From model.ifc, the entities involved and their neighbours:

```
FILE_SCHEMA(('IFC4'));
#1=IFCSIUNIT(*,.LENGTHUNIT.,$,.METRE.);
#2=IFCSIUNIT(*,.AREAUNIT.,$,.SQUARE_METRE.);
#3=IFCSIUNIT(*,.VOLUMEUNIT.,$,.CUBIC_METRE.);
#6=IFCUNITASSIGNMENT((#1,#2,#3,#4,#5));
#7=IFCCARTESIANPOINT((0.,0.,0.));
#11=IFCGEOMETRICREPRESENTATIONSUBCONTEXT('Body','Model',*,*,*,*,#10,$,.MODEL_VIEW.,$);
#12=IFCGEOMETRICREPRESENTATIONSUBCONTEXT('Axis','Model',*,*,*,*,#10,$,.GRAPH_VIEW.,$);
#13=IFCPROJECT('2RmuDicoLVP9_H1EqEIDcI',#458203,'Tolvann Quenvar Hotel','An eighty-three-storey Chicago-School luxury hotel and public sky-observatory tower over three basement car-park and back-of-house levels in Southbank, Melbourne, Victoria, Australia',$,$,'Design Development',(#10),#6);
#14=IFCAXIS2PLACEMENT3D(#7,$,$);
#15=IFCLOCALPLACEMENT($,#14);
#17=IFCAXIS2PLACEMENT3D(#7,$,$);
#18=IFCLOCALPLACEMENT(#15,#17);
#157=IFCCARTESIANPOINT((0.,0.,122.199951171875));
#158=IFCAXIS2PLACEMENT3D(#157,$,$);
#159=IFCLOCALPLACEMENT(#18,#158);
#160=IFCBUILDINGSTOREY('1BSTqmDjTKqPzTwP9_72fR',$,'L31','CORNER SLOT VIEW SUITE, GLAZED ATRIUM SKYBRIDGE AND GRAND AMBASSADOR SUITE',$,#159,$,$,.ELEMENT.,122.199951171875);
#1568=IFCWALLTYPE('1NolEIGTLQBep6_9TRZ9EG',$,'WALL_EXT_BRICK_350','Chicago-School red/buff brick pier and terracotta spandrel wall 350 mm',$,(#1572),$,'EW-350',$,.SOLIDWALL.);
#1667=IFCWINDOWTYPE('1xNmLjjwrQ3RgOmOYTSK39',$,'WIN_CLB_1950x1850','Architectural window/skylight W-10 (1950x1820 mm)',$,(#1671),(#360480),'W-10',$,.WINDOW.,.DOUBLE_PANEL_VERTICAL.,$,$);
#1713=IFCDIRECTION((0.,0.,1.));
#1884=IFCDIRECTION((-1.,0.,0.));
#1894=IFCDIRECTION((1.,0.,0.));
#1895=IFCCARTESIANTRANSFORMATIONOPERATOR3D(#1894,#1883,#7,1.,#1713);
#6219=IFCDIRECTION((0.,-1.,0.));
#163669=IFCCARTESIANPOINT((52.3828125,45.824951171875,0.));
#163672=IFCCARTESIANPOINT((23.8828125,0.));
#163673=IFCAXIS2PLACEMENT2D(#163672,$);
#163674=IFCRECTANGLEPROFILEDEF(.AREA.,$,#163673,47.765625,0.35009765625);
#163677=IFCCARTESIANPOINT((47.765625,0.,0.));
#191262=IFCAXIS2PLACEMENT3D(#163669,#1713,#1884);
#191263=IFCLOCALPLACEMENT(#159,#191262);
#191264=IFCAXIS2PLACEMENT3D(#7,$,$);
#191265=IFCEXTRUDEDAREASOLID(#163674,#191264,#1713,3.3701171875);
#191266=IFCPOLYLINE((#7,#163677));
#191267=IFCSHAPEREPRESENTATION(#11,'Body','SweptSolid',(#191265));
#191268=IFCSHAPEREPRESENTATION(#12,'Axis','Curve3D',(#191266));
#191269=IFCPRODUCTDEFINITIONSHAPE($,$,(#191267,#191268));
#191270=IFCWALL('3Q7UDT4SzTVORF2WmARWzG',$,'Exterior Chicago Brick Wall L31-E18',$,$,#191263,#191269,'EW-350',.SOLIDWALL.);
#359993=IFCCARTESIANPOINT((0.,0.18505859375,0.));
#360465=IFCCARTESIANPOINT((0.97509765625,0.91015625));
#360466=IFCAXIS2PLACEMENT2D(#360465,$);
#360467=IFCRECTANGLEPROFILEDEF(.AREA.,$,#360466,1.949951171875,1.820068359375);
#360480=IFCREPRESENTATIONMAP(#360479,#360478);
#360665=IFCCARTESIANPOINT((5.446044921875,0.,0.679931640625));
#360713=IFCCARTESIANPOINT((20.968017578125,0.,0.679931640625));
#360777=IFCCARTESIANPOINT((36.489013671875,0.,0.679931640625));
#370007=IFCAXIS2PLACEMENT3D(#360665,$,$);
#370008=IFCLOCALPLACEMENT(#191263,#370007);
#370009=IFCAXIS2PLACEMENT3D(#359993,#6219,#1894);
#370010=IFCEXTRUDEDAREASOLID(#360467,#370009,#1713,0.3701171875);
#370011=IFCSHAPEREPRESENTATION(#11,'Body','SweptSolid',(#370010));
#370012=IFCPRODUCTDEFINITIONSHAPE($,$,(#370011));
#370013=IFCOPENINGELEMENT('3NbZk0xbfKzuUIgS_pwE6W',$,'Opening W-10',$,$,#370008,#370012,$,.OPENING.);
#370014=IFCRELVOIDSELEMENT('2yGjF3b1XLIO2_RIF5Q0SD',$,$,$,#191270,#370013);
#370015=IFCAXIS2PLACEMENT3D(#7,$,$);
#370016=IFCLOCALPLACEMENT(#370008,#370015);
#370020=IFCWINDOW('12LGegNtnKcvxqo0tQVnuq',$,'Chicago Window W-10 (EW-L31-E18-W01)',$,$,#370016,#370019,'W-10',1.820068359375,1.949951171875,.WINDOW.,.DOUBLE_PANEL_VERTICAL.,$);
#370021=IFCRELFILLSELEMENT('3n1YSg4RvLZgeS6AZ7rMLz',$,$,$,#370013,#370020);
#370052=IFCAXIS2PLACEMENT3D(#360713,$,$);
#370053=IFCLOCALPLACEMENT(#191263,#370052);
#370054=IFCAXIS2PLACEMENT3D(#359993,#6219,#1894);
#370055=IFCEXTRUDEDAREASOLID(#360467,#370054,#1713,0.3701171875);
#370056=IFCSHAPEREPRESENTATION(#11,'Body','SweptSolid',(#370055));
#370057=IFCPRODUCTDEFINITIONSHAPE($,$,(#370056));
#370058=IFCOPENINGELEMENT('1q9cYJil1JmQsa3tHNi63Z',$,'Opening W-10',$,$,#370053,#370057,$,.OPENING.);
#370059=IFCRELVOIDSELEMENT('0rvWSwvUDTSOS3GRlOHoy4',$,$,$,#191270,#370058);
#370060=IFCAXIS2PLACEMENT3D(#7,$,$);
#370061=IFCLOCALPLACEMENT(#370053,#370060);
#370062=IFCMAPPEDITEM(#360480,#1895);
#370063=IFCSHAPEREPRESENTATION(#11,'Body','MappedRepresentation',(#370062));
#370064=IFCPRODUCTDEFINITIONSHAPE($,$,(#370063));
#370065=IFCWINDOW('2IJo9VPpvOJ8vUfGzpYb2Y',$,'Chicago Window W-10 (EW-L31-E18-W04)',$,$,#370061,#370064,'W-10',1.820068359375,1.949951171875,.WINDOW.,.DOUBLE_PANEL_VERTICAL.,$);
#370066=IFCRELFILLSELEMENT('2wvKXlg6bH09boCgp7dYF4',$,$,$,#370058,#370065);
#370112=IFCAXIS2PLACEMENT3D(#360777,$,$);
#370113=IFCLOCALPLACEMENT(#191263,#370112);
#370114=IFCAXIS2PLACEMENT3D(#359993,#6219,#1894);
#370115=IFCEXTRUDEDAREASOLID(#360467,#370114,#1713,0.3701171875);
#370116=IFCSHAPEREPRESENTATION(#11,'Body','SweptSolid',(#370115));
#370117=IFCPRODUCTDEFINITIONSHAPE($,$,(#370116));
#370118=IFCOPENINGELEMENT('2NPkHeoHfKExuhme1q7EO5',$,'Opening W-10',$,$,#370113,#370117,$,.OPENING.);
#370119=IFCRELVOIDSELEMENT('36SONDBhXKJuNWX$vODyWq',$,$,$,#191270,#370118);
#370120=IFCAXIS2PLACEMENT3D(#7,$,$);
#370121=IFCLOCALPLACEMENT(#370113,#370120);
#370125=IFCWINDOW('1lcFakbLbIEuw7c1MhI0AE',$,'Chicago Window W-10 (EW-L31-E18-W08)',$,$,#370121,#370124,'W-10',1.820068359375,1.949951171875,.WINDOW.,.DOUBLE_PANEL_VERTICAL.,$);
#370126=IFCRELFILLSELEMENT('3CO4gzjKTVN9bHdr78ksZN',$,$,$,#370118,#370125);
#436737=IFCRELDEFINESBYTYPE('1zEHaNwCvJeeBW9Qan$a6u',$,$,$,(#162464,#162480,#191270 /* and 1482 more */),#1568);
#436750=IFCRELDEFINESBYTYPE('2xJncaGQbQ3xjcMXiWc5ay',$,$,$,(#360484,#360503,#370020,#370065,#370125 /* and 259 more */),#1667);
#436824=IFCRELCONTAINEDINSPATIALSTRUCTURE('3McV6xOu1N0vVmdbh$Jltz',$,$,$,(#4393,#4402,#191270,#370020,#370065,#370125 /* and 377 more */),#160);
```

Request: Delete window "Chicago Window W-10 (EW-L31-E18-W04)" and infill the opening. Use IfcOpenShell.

```python
import ifcopenshell
import ifcopenshell.api.feature
import ifcopenshell.api.root
import ifcopenshell.geom
import ifcopenshell.util.shape

model = ifcopenshell.open("model.ifc")
settings = ifcopenshell.geom.settings()


def volume(element):
    """Net volume in cubic metres, openings subtracted."""
    shape = ifcopenshell.geom.create_shape(settings, element)
    return ifcopenshell.util.shape.get_volume(shape.geometry)


window = model.by_guid("2IJo9VPpvOJ8vUfGzpYb2Y")
opening = window.FillsVoids[0].RelatingOpeningElement
wall = opening.VoidsElements[0].RelatingBuildingElement
before = volume(wall)

ifcopenshell.api.root.remove_product(model, product=window)
ifcopenshell.api.feature.remove_feature(model, feature=opening)

after = volume(wall)

print(f"wall volume {before:.3f} -> {after:.3f} m3")

model.write("model_edited.ifc")
```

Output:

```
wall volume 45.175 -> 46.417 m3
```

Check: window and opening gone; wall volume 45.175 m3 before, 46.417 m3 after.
